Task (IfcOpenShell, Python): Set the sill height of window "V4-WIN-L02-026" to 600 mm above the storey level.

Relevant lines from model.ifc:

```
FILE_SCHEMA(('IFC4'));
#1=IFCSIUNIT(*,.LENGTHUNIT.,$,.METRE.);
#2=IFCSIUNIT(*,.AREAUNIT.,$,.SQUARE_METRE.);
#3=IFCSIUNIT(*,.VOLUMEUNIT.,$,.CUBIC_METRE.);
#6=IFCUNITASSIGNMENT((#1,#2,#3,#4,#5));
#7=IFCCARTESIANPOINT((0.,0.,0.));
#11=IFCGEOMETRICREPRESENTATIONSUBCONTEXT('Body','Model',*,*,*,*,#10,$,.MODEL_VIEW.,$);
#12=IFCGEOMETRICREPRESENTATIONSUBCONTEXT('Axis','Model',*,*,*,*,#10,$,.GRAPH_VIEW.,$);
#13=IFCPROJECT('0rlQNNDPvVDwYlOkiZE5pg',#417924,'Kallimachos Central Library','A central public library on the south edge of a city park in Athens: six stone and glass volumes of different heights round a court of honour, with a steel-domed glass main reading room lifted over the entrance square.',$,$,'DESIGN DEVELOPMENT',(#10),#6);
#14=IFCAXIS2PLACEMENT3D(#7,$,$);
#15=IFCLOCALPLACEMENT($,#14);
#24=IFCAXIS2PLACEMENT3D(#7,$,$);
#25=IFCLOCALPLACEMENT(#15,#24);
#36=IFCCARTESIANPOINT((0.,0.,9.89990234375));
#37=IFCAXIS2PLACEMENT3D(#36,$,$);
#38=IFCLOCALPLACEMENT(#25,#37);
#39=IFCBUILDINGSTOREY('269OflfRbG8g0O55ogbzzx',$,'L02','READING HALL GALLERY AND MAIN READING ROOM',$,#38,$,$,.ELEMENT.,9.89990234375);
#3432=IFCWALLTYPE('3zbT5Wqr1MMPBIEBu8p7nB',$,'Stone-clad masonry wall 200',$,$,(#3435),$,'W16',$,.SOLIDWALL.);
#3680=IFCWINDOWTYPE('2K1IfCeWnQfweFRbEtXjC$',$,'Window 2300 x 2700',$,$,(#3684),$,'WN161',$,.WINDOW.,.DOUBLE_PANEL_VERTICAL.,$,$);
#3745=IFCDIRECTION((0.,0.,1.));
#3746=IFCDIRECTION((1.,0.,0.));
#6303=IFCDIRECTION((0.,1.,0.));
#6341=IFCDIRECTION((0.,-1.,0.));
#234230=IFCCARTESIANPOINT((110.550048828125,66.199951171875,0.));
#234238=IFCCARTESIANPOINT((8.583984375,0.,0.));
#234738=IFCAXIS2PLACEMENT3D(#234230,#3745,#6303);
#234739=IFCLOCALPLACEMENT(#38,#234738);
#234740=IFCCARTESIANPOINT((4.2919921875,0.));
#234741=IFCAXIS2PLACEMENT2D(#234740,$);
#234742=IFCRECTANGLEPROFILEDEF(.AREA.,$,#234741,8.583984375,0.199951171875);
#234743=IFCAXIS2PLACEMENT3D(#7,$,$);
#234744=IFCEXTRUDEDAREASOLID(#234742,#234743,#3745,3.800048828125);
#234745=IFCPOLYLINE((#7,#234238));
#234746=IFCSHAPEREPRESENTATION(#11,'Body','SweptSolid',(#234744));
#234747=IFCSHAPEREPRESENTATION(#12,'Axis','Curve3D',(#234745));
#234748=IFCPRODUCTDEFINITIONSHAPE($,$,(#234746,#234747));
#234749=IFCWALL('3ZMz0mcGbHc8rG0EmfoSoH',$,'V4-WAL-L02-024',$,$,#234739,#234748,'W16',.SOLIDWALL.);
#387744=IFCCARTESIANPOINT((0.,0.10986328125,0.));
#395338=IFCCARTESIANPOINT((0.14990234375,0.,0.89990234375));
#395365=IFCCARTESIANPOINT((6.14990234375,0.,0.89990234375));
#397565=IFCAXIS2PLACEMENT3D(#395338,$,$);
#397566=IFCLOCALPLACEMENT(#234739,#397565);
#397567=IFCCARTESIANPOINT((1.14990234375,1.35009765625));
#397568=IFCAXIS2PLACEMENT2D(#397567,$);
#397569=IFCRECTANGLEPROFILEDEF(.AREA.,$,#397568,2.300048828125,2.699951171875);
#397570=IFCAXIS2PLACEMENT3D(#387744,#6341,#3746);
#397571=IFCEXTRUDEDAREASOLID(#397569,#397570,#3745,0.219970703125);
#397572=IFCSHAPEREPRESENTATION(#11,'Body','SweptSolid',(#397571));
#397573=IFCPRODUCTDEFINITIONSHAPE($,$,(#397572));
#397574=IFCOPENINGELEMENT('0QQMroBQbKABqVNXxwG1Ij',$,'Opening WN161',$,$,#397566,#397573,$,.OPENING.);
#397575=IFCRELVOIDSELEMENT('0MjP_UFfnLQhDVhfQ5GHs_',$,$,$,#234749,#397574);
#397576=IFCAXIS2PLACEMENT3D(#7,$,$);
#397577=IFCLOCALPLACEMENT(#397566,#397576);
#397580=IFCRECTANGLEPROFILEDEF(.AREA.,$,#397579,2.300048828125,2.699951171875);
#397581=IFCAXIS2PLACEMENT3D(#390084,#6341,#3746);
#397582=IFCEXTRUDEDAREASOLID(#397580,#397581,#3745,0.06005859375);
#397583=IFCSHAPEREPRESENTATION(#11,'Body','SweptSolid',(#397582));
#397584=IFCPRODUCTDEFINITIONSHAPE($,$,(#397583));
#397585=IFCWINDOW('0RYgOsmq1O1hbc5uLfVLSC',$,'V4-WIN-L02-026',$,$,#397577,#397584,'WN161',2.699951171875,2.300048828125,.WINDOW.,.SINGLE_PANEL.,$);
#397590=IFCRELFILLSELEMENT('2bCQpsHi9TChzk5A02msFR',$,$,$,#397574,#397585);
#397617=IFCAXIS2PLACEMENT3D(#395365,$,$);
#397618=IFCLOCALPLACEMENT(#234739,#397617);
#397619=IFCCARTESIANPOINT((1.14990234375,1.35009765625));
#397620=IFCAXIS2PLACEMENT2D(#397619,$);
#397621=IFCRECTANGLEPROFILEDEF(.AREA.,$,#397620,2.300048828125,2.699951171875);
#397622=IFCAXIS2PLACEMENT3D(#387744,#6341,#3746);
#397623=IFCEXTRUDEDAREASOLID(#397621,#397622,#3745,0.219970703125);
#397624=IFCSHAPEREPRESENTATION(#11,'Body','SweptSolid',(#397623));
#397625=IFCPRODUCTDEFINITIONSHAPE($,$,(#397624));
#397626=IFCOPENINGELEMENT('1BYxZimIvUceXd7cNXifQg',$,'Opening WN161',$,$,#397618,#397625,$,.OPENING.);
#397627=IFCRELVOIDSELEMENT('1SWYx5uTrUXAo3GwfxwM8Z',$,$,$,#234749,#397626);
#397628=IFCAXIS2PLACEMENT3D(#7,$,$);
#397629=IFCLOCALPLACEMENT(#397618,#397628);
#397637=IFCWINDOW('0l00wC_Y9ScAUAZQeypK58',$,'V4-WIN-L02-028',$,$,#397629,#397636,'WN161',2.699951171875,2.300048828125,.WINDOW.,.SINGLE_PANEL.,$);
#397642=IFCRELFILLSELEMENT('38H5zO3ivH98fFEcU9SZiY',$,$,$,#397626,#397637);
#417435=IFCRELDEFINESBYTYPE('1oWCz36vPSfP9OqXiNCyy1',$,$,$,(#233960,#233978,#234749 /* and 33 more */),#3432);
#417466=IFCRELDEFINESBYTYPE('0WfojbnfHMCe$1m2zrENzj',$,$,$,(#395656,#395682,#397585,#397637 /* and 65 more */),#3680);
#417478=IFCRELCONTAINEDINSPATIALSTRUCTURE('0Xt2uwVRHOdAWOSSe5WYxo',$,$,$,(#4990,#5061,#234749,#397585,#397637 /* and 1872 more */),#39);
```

```python
import numpy as np
import ifcopenshell
import ifcopenshell.api.geometry
import ifcopenshell.geom
import ifcopenshell.util.element
import ifcopenshell.util.placement
import ifcopenshell.util.shape
import ifcopenshell.util.unit

model = ifcopenshell.open("model.ifc")
unit_scale = ifcopenshell.util.unit.calculate_unit_scale(model)

window = model.by_id(397585)
opening = window.FillsVoids[0].RelatingOpeningElement
storey = ifcopenshell.util.element.get_container(window, ifc_class="IfcBuildingStorey")
level = ifcopenshell.util.placement.get_local_placement(storey.ObjectPlacement)[2, 3]

# The opening's origin need not be at the sill, so measure its lowest point.
shape = ifcopenshell.geom.create_shape(ifcopenshell.geom.settings(), opening)
bottom = ifcopenshell.util.shape.get_shape_bottom_elevation(shape, shape.geometry) / unit_scale
dz = level + 0.6 - bottom

shift = np.array([0.0, 0.0, dz])
# The window is placed relative to its opening, so it follows when the opening moves.
matrix = ifcopenshell.util.placement.get_local_placement(opening.ObjectPlacement)
matrix[:3, 3] += shift
ifcopenshell.api.geometry.edit_object_placement(
    model, product=opening, matrix=matrix, is_si=False, should_transform_children=True
)

print(f"moved by {dz * unit_scale:+.3f} m")

model.write("model_v2.ifc")
```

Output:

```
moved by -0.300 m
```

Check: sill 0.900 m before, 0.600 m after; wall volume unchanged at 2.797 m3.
